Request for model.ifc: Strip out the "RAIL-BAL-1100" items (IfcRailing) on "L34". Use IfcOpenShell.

First a look at what the model holds.

```python
import ifcopenshell
import ifcopenshell.util.element

model = ifcopenshell.open("model.ifc")
print(model.schema)
storey = next(s for s in model.by_type("IfcBuildingStorey") if s.Name == "L34")
railings = [e for e in ifcopenshell.util.element.get_decomposition(storey) if e.is_a("IfcRailing")]
seen = {}
for e in railings:
    element_type = ifcopenshell.util.element.get_type(e)
    name = element_type.Name if element_type not in (None, e) else None
    seen[name] = seen.get(name, 0) + 1
for name, count in sorted(seen.items(), key=str):
    print(count, "x", name)
```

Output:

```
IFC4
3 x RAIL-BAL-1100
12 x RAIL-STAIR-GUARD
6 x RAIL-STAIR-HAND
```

```python
import ifcopenshell
import ifcopenshell.api.root
import ifcopenshell.util.element

model = ifcopenshell.open("model.ifc")

storey = next(s for s in model.by_type("IfcBuildingStorey") if s.Name == "L34")
railings = [e for e in ifcopenshell.util.element.get_decomposition(storey) if e.is_a("IfcRailing")]
targets = [e for e in railings if (t := ifcopenshell.util.element.get_type(e)) not in (None, e) and t.Name == "RAIL-BAL-1100"]

for e in targets:
    ifcopenshell.api.root.remove_product(model, product=e)
print(len(targets), "removed")

model.write("model_updated.ifc")
```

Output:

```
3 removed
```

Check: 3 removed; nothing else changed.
